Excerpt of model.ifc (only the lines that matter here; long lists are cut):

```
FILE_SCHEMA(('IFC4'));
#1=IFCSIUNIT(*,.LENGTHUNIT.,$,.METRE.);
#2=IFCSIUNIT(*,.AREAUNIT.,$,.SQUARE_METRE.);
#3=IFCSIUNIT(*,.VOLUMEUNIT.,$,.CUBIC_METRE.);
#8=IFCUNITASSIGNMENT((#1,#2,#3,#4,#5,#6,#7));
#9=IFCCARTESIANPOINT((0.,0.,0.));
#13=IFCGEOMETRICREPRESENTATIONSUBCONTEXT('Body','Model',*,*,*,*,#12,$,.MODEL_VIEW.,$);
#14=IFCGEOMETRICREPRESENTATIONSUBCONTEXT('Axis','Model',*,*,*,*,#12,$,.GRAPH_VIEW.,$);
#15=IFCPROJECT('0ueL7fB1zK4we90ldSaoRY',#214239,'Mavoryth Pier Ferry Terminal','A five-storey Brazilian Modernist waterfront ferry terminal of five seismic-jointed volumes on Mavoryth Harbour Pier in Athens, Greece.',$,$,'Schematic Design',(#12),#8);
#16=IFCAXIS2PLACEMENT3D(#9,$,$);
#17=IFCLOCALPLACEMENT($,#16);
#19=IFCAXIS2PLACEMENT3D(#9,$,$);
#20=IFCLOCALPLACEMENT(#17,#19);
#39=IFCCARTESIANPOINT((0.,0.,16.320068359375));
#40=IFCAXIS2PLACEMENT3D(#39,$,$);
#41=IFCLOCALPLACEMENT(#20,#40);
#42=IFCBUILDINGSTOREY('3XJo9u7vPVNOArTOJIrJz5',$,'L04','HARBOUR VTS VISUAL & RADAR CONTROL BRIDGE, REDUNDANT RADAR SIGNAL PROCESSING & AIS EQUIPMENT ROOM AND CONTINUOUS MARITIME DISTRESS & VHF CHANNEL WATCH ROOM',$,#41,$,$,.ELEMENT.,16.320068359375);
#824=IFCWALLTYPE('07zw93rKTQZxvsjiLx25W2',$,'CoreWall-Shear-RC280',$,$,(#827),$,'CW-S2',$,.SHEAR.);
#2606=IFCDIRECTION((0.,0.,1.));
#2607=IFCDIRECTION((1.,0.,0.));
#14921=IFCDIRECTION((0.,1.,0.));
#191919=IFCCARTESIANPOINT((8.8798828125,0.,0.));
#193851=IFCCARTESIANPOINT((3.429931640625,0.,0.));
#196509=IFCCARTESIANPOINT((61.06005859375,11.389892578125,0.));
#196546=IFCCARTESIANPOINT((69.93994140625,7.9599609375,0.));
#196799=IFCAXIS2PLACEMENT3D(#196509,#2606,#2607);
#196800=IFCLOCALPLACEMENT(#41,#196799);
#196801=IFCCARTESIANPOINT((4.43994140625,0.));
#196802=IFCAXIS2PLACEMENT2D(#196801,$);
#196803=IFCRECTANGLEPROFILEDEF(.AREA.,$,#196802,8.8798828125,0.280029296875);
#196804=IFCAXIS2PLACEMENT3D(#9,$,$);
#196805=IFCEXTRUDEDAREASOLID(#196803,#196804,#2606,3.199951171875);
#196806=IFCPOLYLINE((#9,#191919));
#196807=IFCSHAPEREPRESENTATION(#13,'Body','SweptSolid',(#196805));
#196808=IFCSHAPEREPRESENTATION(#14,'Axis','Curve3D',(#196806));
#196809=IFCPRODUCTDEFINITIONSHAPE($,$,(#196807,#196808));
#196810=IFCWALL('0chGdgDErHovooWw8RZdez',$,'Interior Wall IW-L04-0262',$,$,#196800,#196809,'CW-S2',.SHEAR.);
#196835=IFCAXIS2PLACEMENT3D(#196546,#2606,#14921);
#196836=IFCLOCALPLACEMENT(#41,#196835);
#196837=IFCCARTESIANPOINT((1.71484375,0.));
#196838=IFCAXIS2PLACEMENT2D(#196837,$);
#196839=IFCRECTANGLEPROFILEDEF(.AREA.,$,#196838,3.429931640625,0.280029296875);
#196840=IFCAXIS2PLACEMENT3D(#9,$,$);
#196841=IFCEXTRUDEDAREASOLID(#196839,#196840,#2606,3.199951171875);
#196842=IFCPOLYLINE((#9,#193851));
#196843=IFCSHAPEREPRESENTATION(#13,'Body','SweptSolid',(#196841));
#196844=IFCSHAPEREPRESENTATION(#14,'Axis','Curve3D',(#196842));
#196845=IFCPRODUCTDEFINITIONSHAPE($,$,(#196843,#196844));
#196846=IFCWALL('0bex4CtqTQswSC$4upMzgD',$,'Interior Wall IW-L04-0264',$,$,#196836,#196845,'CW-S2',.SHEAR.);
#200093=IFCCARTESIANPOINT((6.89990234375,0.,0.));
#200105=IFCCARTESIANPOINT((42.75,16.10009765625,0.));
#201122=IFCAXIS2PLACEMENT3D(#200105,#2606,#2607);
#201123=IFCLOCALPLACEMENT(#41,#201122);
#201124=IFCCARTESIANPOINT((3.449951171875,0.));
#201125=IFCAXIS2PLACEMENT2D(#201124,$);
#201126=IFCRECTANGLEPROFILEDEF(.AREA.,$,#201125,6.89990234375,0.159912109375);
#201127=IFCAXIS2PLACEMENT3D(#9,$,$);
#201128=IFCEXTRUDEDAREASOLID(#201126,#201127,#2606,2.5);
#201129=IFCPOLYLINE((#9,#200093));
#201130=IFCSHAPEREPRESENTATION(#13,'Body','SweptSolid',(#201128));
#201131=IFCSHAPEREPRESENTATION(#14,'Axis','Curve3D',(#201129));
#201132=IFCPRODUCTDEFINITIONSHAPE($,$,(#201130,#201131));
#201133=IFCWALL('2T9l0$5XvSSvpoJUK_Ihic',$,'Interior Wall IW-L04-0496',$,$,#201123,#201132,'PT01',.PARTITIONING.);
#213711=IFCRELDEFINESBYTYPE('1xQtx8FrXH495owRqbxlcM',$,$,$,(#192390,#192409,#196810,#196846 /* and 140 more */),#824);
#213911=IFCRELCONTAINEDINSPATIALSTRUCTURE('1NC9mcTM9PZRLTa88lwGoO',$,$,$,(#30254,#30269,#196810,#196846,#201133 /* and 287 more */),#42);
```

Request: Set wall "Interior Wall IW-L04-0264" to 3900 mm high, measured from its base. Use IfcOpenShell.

```python
import ifcopenshell
import ifcopenshell.geom
import ifcopenshell.util.representation
import ifcopenshell.util.shape

model = ifcopenshell.open("model.ifc")
settings = ifcopenshell.geom.settings()


def volume(element):
    """Net volume in cubic metres, openings subtracted."""
    shape = ifcopenshell.geom.create_shape(settings, element)
    return ifcopenshell.util.shape.get_volume(shape.geometry)


wall = model.by_guid("0bex4CtqTQswSC$4upMzgD")
before = volume(wall)

body = ifcopenshell.util.representation.get_representation(wall, "Model", "Body")
solid = body.Items[0]
old_height = solid.Depth
solid.Depth = 3.9
after = volume(wall)

print(f"height {old_height:g} -> {solid.Depth:g}, volume {before:.3f} -> {after:.3f} m3")

model.write("model_edited.ifc")
```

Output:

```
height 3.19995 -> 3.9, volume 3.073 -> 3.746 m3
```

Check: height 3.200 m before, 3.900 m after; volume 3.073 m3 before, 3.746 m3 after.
